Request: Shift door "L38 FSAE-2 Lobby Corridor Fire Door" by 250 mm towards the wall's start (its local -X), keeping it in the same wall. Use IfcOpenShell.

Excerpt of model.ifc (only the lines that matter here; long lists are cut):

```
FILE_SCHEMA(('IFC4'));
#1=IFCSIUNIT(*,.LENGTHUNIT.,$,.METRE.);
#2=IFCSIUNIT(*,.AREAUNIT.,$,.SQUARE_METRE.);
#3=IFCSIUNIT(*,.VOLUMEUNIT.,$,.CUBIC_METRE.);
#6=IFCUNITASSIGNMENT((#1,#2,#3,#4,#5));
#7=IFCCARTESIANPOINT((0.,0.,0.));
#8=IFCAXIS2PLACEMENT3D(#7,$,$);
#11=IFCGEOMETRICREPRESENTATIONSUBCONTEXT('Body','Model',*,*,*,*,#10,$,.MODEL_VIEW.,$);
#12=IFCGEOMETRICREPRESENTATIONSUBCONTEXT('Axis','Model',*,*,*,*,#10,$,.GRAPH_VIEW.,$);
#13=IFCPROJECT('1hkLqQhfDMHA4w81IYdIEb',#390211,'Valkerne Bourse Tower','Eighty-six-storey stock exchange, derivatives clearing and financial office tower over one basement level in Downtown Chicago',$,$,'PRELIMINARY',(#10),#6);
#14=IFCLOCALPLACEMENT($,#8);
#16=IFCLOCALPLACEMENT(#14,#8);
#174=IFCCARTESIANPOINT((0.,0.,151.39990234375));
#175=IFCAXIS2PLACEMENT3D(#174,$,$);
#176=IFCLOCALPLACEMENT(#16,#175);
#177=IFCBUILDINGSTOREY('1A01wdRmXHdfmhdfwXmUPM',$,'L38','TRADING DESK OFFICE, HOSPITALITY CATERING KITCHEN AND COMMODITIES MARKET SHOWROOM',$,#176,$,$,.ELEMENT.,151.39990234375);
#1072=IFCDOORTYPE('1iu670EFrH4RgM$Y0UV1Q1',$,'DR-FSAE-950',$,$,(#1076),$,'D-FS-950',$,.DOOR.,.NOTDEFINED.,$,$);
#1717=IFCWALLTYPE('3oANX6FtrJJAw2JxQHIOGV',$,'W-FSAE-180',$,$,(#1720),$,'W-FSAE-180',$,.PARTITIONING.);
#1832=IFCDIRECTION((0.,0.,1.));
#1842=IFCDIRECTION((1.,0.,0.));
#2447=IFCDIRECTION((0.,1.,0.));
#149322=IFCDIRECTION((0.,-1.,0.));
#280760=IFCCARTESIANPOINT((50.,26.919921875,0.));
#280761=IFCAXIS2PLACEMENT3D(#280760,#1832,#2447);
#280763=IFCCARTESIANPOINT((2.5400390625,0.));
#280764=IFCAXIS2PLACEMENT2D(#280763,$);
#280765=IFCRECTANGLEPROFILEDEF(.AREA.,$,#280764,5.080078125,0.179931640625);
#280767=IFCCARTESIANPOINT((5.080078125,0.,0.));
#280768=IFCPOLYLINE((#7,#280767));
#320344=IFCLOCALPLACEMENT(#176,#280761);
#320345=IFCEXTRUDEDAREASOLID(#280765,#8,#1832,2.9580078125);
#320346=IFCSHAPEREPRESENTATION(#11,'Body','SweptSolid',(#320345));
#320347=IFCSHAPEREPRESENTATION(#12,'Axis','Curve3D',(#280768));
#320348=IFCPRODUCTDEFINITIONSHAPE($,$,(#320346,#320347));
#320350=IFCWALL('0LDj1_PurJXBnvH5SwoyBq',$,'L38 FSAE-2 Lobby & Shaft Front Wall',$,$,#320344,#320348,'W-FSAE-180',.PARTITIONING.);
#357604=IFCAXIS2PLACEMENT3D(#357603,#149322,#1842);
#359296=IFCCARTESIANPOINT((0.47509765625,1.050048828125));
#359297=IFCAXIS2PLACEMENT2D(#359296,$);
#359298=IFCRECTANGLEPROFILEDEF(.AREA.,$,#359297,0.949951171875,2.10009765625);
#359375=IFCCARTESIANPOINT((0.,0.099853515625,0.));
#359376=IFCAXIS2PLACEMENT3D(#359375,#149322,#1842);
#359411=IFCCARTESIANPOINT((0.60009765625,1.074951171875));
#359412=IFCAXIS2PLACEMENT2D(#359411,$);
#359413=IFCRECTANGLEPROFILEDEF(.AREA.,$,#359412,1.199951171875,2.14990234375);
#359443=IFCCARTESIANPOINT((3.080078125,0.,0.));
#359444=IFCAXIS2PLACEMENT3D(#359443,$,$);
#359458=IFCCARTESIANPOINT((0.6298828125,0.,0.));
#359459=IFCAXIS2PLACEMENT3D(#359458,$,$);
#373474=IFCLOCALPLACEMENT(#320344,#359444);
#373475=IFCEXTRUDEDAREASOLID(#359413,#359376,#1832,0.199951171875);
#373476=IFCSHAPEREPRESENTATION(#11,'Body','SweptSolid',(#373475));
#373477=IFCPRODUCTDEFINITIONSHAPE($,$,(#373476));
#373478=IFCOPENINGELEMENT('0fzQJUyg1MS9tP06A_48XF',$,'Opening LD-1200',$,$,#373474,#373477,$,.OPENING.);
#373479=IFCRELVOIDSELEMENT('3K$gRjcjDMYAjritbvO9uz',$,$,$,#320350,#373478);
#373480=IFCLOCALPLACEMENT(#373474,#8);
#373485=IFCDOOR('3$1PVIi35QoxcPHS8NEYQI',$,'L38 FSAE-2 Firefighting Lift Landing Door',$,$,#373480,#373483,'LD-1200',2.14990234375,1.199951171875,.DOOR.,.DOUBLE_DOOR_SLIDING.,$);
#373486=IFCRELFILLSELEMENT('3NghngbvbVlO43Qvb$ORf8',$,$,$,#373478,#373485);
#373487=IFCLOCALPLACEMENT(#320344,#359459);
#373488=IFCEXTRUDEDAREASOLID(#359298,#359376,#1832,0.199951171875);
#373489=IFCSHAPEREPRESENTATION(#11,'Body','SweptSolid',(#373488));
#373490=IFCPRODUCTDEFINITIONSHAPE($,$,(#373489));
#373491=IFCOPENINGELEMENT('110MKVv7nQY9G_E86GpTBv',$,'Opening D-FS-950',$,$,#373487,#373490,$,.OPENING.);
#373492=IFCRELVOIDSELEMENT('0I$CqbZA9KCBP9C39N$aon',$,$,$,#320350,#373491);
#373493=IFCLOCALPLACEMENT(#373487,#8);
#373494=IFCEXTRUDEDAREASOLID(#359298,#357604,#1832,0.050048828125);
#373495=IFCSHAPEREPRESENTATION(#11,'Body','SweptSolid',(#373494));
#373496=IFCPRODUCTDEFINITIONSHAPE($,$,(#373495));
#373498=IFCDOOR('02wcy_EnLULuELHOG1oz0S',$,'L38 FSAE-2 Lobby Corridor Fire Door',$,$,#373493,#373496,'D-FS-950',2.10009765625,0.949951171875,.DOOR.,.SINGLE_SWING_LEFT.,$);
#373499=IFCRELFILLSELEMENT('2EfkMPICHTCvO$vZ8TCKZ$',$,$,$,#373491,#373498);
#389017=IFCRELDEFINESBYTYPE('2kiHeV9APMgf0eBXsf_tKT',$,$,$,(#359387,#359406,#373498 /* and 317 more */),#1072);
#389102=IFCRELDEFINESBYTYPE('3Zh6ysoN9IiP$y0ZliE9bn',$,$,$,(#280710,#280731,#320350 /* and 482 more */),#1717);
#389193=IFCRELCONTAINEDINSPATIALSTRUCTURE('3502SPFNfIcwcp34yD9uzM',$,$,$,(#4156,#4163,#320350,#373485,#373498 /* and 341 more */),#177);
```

```python
import ifcopenshell
import ifcopenshell.api.geometry
import ifcopenshell.util.placement

model = ifcopenshell.open("model.ifc")

door = model.by_guid("02wcy_EnLULuELHOG1oz0S")
opening = door.FillsVoids[0].RelatingOpeningElement
wall = opening.VoidsElements[0].RelatingBuildingElement

wall_matrix = ifcopenshell.util.placement.get_local_placement(wall.ObjectPlacement)
shift = wall_matrix[:3, 0] * -0.25
before = ifcopenshell.util.placement.get_local_placement(door.ObjectPlacement)[:3, 3].copy()

# The door is placed relative to its opening, so it follows when the opening moves.
matrix = ifcopenshell.util.placement.get_local_placement(opening.ObjectPlacement)
matrix[:3, 3] += shift
ifcopenshell.api.geometry.edit_object_placement(
    model, product=opening, matrix=matrix, is_si=False, should_transform_children=True
)

after = ifcopenshell.util.placement.get_local_placement(door.ObjectPlacement)[:3, 3]
print("door moved by", (after - before).round(3) + 0.0)

model.write("model_rev.ifc")
```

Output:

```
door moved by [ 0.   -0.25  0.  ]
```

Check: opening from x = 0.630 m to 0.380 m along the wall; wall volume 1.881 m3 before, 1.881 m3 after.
